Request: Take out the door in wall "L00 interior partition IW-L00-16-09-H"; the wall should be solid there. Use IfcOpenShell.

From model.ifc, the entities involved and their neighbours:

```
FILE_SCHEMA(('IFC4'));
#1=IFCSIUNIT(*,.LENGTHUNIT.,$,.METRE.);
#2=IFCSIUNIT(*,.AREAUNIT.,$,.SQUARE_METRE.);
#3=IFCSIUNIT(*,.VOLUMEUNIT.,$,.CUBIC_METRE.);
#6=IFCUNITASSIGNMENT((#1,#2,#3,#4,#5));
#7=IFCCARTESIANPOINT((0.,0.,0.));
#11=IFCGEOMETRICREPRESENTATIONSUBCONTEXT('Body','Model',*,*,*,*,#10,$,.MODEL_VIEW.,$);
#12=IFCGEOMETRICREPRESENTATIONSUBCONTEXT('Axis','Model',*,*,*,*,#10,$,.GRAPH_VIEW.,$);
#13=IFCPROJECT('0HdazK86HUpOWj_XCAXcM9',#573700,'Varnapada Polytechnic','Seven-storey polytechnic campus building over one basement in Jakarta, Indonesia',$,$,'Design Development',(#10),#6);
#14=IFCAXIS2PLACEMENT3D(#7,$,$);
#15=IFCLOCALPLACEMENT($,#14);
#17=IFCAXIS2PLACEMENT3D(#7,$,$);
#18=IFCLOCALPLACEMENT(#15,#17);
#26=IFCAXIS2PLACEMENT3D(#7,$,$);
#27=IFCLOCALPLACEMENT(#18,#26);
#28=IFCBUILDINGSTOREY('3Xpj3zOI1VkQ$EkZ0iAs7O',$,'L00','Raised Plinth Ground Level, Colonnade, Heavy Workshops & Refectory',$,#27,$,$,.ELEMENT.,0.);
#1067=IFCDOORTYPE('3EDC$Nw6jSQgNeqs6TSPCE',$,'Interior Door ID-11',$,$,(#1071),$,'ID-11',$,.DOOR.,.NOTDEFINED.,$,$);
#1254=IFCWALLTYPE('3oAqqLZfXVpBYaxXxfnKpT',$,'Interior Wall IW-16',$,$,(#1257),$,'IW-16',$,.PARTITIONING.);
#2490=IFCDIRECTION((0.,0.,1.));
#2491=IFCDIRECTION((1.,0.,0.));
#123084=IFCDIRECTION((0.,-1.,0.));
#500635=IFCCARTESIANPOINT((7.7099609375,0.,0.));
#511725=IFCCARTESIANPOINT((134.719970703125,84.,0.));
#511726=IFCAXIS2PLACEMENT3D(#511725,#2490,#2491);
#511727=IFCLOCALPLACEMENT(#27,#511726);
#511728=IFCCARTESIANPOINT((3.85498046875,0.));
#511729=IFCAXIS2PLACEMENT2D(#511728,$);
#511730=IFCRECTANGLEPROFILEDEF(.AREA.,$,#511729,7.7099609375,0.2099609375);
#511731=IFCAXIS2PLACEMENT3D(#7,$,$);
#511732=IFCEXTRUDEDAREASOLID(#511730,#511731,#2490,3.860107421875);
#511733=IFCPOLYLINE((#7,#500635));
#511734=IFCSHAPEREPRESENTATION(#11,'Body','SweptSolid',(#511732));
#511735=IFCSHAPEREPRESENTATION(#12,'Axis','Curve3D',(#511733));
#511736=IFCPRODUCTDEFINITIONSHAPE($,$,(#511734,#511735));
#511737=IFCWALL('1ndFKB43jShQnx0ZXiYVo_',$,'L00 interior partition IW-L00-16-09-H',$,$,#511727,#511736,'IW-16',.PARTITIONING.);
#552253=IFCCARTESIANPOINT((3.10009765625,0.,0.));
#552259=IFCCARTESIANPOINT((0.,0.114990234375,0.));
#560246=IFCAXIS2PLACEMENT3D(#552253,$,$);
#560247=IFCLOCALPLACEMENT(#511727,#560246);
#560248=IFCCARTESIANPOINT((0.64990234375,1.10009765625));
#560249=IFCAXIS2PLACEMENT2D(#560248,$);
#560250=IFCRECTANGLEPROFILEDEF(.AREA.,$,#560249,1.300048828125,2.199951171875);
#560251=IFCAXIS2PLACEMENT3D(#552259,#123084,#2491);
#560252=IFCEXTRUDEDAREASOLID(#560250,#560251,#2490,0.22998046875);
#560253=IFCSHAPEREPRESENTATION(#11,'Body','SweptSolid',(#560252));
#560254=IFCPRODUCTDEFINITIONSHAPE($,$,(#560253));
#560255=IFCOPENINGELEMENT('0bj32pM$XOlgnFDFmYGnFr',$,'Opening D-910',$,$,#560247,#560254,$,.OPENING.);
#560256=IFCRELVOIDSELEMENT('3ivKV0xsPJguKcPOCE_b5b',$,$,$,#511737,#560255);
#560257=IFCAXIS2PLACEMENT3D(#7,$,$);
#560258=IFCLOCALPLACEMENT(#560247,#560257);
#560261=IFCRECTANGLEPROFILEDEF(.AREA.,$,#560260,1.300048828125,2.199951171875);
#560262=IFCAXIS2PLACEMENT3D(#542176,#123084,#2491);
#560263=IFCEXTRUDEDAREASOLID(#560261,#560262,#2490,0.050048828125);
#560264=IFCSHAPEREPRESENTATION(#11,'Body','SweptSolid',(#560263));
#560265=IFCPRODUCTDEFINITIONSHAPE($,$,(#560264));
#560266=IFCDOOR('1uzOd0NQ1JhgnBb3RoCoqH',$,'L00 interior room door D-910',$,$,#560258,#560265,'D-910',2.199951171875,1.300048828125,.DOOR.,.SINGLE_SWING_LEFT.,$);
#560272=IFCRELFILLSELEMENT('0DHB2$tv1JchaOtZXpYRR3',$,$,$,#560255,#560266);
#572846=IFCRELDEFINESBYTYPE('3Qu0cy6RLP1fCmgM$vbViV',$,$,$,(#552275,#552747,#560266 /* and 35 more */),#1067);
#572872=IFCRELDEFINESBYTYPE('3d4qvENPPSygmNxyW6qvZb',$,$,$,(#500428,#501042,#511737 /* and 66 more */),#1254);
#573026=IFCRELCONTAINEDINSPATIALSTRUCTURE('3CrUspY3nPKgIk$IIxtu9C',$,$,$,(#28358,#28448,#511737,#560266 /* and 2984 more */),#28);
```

```python
import ifcopenshell
import ifcopenshell.api.feature
import ifcopenshell.api.root
import ifcopenshell.geom
import ifcopenshell.util.shape

model = ifcopenshell.open("model.ifc")
settings = ifcopenshell.geom.settings()


def volume(element):
    """Net volume in cubic metres, openings subtracted."""
    shape = ifcopenshell.geom.create_shape(settings, element)
    return ifcopenshell.util.shape.get_volume(shape.geometry)


door = model.by_guid("1uzOd0NQ1JhgnBb3RoCoqH")
opening = door.FillsVoids[0].RelatingOpeningElement
wall = opening.VoidsElements[0].RelatingBuildingElement
before = volume(wall)

ifcopenshell.api.root.remove_product(model, product=door)
ifcopenshell.api.feature.remove_feature(model, feature=opening)

after = volume(wall)

print(f"wall volume {before:.3f} -> {after:.3f} m3")

model.write("model_updated.ifc")
```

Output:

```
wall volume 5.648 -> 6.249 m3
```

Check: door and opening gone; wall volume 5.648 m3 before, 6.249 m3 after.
